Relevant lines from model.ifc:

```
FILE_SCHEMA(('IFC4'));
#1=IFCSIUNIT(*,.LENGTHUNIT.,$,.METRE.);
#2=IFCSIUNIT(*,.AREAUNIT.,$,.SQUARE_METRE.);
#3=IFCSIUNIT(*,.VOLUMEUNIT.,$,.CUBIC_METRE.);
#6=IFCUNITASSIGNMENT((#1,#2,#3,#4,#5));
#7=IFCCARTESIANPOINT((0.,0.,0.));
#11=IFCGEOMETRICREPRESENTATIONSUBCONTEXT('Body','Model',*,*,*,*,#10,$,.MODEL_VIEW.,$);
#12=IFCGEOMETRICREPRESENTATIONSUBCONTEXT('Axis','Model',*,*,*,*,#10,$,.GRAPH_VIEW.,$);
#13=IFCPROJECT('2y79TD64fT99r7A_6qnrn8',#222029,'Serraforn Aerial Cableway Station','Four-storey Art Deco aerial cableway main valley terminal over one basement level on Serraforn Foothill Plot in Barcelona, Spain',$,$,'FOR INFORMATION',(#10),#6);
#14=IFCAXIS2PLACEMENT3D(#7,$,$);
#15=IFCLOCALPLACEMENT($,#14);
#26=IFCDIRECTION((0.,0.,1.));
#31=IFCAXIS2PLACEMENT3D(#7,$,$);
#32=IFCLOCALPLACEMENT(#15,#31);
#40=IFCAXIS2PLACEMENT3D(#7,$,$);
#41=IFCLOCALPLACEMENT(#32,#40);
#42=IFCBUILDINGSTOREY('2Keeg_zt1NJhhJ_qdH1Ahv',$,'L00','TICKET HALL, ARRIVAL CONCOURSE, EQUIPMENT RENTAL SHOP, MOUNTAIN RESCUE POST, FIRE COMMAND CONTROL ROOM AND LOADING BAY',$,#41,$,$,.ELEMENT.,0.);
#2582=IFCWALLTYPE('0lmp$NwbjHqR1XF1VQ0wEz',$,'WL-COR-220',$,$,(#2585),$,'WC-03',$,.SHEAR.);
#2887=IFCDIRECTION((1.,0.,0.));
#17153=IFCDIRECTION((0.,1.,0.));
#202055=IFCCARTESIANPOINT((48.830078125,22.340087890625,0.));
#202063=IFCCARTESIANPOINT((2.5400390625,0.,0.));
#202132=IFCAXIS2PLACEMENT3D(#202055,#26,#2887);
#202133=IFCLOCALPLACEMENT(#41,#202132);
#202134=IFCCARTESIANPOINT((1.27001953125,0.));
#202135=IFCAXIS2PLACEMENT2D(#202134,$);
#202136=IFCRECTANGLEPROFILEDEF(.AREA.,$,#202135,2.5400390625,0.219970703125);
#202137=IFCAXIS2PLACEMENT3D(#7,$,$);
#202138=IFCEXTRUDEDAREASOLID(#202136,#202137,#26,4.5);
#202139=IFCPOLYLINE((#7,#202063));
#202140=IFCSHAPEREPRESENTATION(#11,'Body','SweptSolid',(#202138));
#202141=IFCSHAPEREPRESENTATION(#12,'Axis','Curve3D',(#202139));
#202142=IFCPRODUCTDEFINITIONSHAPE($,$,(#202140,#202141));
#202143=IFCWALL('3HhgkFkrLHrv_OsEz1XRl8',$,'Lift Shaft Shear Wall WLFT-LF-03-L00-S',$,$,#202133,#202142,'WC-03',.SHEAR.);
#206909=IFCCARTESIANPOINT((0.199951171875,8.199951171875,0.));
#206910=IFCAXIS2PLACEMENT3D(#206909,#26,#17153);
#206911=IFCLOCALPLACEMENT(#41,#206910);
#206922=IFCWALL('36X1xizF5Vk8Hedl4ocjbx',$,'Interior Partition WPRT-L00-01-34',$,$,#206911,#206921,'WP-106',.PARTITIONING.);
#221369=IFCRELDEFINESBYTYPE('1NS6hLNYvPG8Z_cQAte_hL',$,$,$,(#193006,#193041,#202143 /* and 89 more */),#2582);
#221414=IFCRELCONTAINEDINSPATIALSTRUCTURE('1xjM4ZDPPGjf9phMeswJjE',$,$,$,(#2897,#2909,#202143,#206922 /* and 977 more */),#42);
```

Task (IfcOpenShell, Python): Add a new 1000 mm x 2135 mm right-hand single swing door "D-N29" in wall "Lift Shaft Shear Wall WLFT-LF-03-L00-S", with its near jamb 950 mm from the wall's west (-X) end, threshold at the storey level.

```python
import numpy as np
import ifcopenshell
import ifcopenshell.api.feature
import ifcopenshell.api.geometry
import ifcopenshell.api.root
import ifcopenshell.api.spatial
import ifcopenshell.geom
import ifcopenshell.util.element
import ifcopenshell.util.placement
import ifcopenshell.util.representation
import ifcopenshell.util.shape
import ifcopenshell.util.unit

model = ifcopenshell.open("model.ifc")
unit_scale = ifcopenshell.util.unit.calculate_unit_scale(model)
settings = ifcopenshell.geom.settings()


def volume(element):
    """Net volume in cubic metres, openings subtracted."""
    shape = ifcopenshell.geom.create_shape(settings, element)
    return ifcopenshell.util.shape.get_volume(shape.geometry)


wall = model.by_guid("3HhgkFkrLHrv_OsEz1XRl8")
storey = ifcopenshell.util.element.get_container(wall, ifc_class="IfcBuildingStorey")
context = ifcopenshell.util.representation.get_context(model, "Model", "Body", "MODEL_VIEW")
before = volume(wall)

width, height, from_end, sill = 1, 2.135, 0.95, 0.0  # metres

# The wall runs along its own X axis, and the end named is its -X end.
wall_shape = ifcopenshell.geom.create_shape(settings, wall)
x, y, z = ifcopenshell.util.shape.get_vertices(wall_shape.geometry).T
start = x.min() + from_end
face, thickness = float(y.min()), float(y.max() - y.min())
wall_matrix = ifcopenshell.util.placement.get_local_placement(wall.ObjectPlacement)
level = ifcopenshell.util.placement.get_local_placement(storey.ObjectPlacement)[2, 3]


def in_wall(x, y):
    """Placement at x, y metres in the wall's axes, at sill height."""
    matrix = wall_matrix.copy()
    matrix[:, 3] = wall_matrix @ np.array([x / unit_scale, y / unit_scale, 0.0, 1.0])
    matrix[2, 3] = level + sill / unit_scale
    return matrix


# Opening: a box that overshoots both wall faces by 50 mm.
opening = ifcopenshell.api.root.create_entity(model, ifc_class="IfcOpeningElement", predefined_type="OPENING")
box = ifcopenshell.api.geometry.add_wall_representation(
    model, context=context, length=width, height=height, thickness=thickness + 0.1
)
ifcopenshell.api.geometry.assign_representation(model, product=opening, representation=box)
ifcopenshell.api.geometry.edit_object_placement(model, product=opening, matrix=in_wall(start, face - 0.05), is_si=False)
ifcopenshell.api.feature.add_feature(model, feature=opening, element=wall)

door = ifcopenshell.api.root.create_entity(model, ifc_class="IfcDoor", name="D-N29", predefined_type="DOOR")
door.OverallWidth, door.OverallHeight = width / unit_scale, height / unit_scale
door.OperationType = "SINGLE_SWING_RIGHT"
body = ifcopenshell.api.geometry.add_door_representation(
    model,
    context=context,
    overall_width=door.OverallWidth,
    overall_height=door.OverallHeight,
    operation_type="SINGLE_SWING_RIGHT",
    lining_properties={"LiningDepth": thickness / unit_scale, "ThresholdDepth": thickness / unit_scale},
)
ifcopenshell.api.geometry.assign_representation(model, product=door, representation=body)
ifcopenshell.api.spatial.assign_container(model, products=[door], relating_structure=storey)
ifcopenshell.api.feature.add_filling(model, opening=opening, element=door)

# The lining spans the wall, so the door starts at the wall face.
ifcopenshell.api.geometry.edit_object_placement(model, product=door, matrix=in_wall(start, face), is_si=False)

after = volume(wall)

print(f"wall volume {before:.3f} -> {after:.3f} m3")

model.write("model_rev.ifc")
```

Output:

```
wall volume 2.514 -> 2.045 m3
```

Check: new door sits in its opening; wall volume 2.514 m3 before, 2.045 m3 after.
